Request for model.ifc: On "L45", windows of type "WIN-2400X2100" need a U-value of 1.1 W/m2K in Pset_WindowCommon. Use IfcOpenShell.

First a look at what the model holds.

```python
import ifcopenshell
import ifcopenshell.util.element

model = ifcopenshell.open("model.ifc")
print(model.schema)
storey = next(s for s in model.by_type("IfcBuildingStorey") if s.Name == "L45")
windows = [e for e in ifcopenshell.util.element.get_decomposition(storey) if e.is_a("IfcWindow")]
seen = {}
for e in windows:
    element_type = ifcopenshell.util.element.get_type(e)
    key = (element_type.Name if element_type != e and element_type else None, ifcopenshell.util.element.get_pset(e, "Pset_WindowCommon", "ThermalTransmittance"))
    seen[key] = seen.get(key, 0) + 1
for (name, value), count in sorted(seen.items(), key=str):
    print(count, "x", name, "|", value)
```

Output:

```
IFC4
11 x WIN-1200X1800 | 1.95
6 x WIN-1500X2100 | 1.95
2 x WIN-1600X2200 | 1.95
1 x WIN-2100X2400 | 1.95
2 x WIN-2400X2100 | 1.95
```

```python
import ifcopenshell
import ifcopenshell.api.pset
import ifcopenshell.util.element

model = ifcopenshell.open("model.ifc")

storey = next(s for s in model.by_type("IfcBuildingStorey") if s.Name == "L45")
windows = [e for e in ifcopenshell.util.element.get_decomposition(storey) if e.is_a("IfcWindow")]

count = 0
for e in windows:
    element_type = ifcopenshell.util.element.get_type(e)
    if element_type in (None, e) or element_type.Name != "WIN-2400X2100":
        continue
    # add_pset returns the element's existing set when there is one.
    pset = ifcopenshell.api.pset.add_pset(model, product=e, name="Pset_WindowCommon")
    ifcopenshell.api.pset.edit_pset(model, pset=pset, properties={"ThermalTransmittance": 1.1})
    count += 1

print(count, "windows updated")

model.write("model_edited.ifc")
```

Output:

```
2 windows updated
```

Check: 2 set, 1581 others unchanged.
